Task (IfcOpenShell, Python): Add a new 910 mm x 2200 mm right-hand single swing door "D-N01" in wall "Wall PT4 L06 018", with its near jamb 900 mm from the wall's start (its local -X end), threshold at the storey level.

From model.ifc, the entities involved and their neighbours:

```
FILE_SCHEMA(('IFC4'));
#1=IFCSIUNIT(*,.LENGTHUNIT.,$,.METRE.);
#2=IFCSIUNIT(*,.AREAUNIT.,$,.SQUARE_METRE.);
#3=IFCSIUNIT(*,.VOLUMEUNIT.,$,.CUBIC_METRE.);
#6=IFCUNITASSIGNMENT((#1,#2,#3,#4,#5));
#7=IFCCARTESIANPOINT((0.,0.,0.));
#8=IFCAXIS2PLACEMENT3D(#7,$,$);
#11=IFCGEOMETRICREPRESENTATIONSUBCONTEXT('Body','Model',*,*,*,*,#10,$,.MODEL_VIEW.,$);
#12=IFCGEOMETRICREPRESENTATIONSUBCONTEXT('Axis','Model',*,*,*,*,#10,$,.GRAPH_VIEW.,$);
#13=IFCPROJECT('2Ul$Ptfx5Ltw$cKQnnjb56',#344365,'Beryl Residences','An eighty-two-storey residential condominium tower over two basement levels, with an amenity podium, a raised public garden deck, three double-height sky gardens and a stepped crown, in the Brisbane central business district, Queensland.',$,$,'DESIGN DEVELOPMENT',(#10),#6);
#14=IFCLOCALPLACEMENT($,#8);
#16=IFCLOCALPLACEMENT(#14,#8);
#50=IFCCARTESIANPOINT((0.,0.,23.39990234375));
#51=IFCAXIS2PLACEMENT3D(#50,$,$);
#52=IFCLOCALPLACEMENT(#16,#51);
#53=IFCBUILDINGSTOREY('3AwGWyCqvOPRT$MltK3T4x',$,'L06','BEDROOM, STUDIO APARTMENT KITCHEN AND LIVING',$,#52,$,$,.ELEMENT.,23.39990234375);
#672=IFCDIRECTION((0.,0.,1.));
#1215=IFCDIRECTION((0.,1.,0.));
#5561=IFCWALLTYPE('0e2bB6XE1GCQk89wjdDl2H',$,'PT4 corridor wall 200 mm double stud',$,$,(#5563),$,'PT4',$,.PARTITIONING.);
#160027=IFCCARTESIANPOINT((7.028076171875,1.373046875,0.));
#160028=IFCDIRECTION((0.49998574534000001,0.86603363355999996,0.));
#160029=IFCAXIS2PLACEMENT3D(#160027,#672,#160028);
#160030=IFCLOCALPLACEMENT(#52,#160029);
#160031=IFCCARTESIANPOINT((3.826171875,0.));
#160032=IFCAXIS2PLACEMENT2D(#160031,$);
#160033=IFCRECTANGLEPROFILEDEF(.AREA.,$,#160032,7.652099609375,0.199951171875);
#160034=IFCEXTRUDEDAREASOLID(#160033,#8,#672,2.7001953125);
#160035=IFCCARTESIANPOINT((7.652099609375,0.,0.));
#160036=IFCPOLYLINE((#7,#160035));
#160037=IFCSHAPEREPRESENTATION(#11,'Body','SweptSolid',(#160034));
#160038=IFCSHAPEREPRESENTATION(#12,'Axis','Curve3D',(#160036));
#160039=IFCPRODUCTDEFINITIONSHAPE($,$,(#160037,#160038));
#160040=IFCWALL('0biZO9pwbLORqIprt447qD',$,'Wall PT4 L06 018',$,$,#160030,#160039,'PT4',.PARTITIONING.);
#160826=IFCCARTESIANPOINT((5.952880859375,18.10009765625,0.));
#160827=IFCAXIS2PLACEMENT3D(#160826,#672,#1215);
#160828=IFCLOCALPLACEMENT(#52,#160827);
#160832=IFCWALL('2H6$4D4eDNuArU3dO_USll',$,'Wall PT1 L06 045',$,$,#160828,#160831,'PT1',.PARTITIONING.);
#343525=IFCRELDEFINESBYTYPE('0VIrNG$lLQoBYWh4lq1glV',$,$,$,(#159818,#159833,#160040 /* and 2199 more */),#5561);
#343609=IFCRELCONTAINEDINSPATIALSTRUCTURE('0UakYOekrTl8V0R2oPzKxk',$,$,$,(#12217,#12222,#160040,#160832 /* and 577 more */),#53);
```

```python
import numpy as np
import ifcopenshell
import ifcopenshell.api.feature
import ifcopenshell.api.geometry
import ifcopenshell.api.root
import ifcopenshell.api.spatial
import ifcopenshell.geom
import ifcopenshell.util.element
import ifcopenshell.util.placement
import ifcopenshell.util.representation
import ifcopenshell.util.shape
import ifcopenshell.util.unit

model = ifcopenshell.open("model.ifc")
unit_scale = ifcopenshell.util.unit.calculate_unit_scale(model)
settings = ifcopenshell.geom.settings()


def volume(element):
    """Net volume in cubic metres, openings subtracted."""
    shape = ifcopenshell.geom.create_shape(settings, element)
    return ifcopenshell.util.shape.get_volume(shape.geometry)


wall = model.by_id(160040)
storey = ifcopenshell.util.element.get_container(wall, ifc_class="IfcBuildingStorey")
context = ifcopenshell.util.representation.get_context(model, "Model", "Body", "MODEL_VIEW")
before = volume(wall)

width, height, from_end, sill = 0.91, 2.2, 0.9, 0.0  # metres

# The wall runs along its own X axis, and the end named is its -X end.
wall_shape = ifcopenshell.geom.create_shape(settings, wall)
x, y, z = ifcopenshell.util.shape.get_vertices(wall_shape.geometry).T
start = x.min() + from_end
face, thickness = float(y.min()), float(y.max() - y.min())
wall_matrix = ifcopenshell.util.placement.get_local_placement(wall.ObjectPlacement)
level = ifcopenshell.util.placement.get_local_placement(storey.ObjectPlacement)[2, 3]


def in_wall(x, y):
    """Placement at x, y metres in the wall's axes, at sill height."""
    matrix = wall_matrix.copy()
    matrix[:, 3] = wall_matrix @ np.array([x / unit_scale, y / unit_scale, 0.0, 1.0])
    matrix[2, 3] = level + sill / unit_scale
    return matrix


# Opening: a box that overshoots both wall faces by 50 mm.
opening = ifcopenshell.api.root.create_entity(model, ifc_class="IfcOpeningElement", predefined_type="OPENING")
box = ifcopenshell.api.geometry.add_wall_representation(
    model, context=context, length=width, height=height, thickness=thickness + 0.1
)
ifcopenshell.api.geometry.assign_representation(model, product=opening, representation=box)
ifcopenshell.api.geometry.edit_object_placement(model, product=opening, matrix=in_wall(start, face - 0.05), is_si=False)
ifcopenshell.api.feature.add_feature(model, feature=opening, element=wall)

door = ifcopenshell.api.root.create_entity(model, ifc_class="IfcDoor", name="D-N01", predefined_type="DOOR")
door.OverallWidth, door.OverallHeight = width / unit_scale, height / unit_scale
door.OperationType = "SINGLE_SWING_RIGHT"
body = ifcopenshell.api.geometry.add_door_representation(
    model,
    context=context,
    overall_width=door.OverallWidth,
    overall_height=door.OverallHeight,
    operation_type="SINGLE_SWING_RIGHT",
    lining_properties={"LiningDepth": thickness / unit_scale, "ThresholdDepth": thickness / unit_scale},
)
ifcopenshell.api.geometry.assign_representation(model, product=door, representation=body)
ifcopenshell.api.spatial.assign_container(model, products=[door], relating_structure=storey)
ifcopenshell.api.feature.add_filling(model, opening=opening, element=door)

# The lining spans the wall, so the door starts at the wall face.
ifcopenshell.api.geometry.edit_object_placement(model, product=door, matrix=in_wall(start, face), is_si=False)

after = volume(wall)

print(f"wall volume {before:.3f} -> {after:.3f} m3")

model.write("model_edited.ifc")
```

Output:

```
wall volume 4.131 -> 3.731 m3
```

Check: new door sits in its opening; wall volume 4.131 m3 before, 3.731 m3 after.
